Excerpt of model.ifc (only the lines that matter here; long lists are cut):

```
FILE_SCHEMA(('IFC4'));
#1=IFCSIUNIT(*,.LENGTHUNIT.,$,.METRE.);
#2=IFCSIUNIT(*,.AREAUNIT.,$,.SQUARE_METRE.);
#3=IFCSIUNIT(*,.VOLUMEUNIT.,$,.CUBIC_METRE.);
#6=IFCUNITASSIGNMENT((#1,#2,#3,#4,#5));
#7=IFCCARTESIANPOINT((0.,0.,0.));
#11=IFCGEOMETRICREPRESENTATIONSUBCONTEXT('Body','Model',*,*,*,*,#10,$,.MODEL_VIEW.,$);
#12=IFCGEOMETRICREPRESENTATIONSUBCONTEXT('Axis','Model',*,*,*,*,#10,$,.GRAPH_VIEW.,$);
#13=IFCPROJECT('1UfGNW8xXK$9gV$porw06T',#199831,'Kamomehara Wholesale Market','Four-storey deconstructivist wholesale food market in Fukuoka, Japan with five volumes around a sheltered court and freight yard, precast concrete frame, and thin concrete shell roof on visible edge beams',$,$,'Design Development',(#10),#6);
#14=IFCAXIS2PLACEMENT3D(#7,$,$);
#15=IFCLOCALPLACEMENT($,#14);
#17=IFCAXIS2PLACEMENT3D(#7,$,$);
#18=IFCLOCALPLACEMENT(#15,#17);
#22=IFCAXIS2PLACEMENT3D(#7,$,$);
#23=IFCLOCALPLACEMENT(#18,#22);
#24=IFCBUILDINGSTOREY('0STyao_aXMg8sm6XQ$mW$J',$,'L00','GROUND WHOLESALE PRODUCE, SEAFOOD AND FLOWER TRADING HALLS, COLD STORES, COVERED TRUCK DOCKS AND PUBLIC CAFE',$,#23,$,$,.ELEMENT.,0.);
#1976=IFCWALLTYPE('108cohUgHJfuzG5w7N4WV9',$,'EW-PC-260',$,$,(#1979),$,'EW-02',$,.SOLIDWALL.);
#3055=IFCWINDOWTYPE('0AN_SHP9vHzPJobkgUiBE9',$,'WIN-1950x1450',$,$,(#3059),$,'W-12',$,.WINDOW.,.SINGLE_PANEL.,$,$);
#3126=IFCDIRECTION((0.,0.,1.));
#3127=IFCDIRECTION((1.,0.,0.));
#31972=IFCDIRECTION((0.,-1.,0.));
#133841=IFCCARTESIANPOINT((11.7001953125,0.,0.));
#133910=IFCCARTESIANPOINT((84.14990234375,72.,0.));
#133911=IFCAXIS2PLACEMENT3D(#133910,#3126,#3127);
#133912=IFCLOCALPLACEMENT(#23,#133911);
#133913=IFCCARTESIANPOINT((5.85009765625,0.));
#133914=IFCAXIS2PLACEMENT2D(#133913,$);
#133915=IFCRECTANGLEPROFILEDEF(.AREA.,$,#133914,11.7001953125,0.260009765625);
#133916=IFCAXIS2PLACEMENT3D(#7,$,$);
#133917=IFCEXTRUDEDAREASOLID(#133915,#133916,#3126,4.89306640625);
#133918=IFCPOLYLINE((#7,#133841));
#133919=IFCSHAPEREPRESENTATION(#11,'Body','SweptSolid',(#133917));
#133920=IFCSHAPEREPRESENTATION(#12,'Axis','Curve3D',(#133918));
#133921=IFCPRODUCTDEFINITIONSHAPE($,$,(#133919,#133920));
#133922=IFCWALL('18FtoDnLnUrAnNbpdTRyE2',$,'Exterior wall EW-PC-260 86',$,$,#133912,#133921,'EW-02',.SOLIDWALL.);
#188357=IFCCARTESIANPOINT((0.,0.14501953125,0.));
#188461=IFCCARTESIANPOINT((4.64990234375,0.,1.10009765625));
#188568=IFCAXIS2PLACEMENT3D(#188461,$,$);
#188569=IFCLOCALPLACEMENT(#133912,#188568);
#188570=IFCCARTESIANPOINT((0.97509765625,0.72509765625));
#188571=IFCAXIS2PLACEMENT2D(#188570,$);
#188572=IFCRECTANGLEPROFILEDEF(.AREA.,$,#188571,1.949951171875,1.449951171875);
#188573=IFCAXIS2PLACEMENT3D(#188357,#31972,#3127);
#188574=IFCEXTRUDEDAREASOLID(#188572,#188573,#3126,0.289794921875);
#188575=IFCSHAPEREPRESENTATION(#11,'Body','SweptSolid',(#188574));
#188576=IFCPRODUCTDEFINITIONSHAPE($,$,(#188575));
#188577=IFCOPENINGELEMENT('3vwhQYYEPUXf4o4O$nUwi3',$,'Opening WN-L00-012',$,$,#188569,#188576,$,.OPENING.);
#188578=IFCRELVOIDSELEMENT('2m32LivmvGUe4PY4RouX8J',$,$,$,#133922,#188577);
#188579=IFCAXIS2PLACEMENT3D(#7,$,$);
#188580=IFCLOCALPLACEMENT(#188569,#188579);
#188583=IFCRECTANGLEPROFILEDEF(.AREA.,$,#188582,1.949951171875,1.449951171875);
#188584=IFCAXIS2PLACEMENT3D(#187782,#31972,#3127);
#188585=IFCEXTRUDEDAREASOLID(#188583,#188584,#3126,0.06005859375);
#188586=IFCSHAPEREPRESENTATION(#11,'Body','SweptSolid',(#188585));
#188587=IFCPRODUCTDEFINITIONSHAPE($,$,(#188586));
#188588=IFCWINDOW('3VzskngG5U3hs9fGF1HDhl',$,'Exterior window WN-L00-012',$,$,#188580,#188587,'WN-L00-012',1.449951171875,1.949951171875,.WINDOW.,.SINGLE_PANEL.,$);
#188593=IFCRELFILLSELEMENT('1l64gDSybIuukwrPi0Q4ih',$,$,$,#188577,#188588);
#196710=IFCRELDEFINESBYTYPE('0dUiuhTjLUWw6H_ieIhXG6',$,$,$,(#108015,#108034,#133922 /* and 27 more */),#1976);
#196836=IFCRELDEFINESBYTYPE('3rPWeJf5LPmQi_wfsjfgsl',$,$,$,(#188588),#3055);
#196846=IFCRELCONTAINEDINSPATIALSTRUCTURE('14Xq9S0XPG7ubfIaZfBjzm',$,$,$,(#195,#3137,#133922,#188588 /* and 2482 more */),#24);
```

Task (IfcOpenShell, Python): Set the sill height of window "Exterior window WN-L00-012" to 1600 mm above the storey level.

```python
import numpy as np
import ifcopenshell
import ifcopenshell.api.geometry
import ifcopenshell.geom
import ifcopenshell.util.element
import ifcopenshell.util.placement
import ifcopenshell.util.shape
import ifcopenshell.util.unit

model = ifcopenshell.open("model.ifc")
unit_scale = ifcopenshell.util.unit.calculate_unit_scale(model)

window = model.by_guid("3VzskngG5U3hs9fGF1HDhl")
opening = window.FillsVoids[0].RelatingOpeningElement
storey = ifcopenshell.util.element.get_container(window, ifc_class="IfcBuildingStorey")
level = ifcopenshell.util.placement.get_local_placement(storey.ObjectPlacement)[2, 3]

# The opening's origin need not be at the sill, so measure its lowest point.
shape = ifcopenshell.geom.create_shape(ifcopenshell.geom.settings(), opening)
bottom = ifcopenshell.util.shape.get_shape_bottom_elevation(shape, shape.geometry) / unit_scale
dz = level + 1.6 - bottom

shift = np.array([0.0, 0.0, dz])
# The window is placed relative to its opening, so it follows when the opening moves.
matrix = ifcopenshell.util.placement.get_local_placement(opening.ObjectPlacement)
matrix[:3, 3] += shift
ifcopenshell.api.geometry.edit_object_placement(
    model, product=opening, matrix=matrix, is_si=False, should_transform_children=True
)

print(f"moved by {dz * unit_scale:+.3f} m")

model.write("model-out.ifc")
```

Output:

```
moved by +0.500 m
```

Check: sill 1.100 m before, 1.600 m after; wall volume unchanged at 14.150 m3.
